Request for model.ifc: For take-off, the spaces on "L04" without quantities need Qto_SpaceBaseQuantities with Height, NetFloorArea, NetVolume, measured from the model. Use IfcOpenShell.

First a look at what the model holds.

```python
import ifcopenshell
import ifcopenshell.util.element
import ifcopenshell.util.unit

model = ifcopenshell.open("model.ifc")
print(model.schema)
for unit_type in ("LENGTHUNIT", "AREAUNIT", "VOLUMEUNIT"):
    print(unit_type, ifcopenshell.util.unit.calculate_unit_scale(model, unit_type))
storey = next(s for s in model.by_type("IfcBuildingStorey") if s.Name == "L04")
spaces = [e for e in ifcopenshell.util.element.get_decomposition(storey) if e.is_a("IfcSpace")]
for e in sorted(spaces, key=lambda e: e.id()):
    print(e.id(), e.is_a(), e.Name, list(ifcopenshell.util.element.get_psets(e, qtos_only=True)), sep=" | ")
```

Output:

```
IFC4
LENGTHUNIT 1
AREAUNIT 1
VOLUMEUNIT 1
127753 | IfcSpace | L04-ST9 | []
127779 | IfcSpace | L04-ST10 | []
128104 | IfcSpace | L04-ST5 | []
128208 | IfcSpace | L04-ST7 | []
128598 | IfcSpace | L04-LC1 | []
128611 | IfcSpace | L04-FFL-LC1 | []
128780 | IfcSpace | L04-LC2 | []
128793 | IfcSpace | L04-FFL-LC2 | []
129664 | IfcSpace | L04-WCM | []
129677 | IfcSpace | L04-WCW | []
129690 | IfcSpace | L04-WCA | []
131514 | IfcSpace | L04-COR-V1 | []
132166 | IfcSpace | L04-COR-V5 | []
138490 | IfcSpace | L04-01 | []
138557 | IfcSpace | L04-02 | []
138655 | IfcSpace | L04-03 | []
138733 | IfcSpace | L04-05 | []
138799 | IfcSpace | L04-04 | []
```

```python
import ifcopenshell
import ifcopenshell.api.pset
import ifcopenshell.geom
import ifcopenshell.util.element
import ifcopenshell.util.shape
import ifcopenshell.util.unit

model = ifcopenshell.open("model.ifc")
unit_scale = ifcopenshell.util.unit.calculate_unit_scale(model)
area_scale = ifcopenshell.util.unit.calculate_unit_scale(model, "AREAUNIT")
volume_scale = ifcopenshell.util.unit.calculate_unit_scale(model, "VOLUMEUNIT")
settings = ifcopenshell.geom.settings()

storey = next(s for s in model.by_type("IfcBuildingStorey") if s.Name == "L04")
spaces = [e for e in ifcopenshell.util.element.get_decomposition(storey) if e.is_a("IfcSpace")]

for e in sorted(spaces, key=lambda e: e.id()):
    if ifcopenshell.util.element.get_psets(e, qtos_only=True, should_inherit=False):
        continue
    # Geometry comes back in metres, in the element's own axes.
    shape = ifcopenshell.geom.create_shape(settings, e)
    values = {
        "Height": ifcopenshell.util.shape.get_z(shape.geometry) / unit_scale,
        "NetFloorArea": ifcopenshell.util.shape.get_footprint_area(shape.geometry) / area_scale,
        "NetVolume": ifcopenshell.util.shape.get_volume(shape.geometry) / volume_scale,
    }
    qto = ifcopenshell.api.pset.add_qto(model, product=e, name="Qto_SpaceBaseQuantities")
    ifcopenshell.api.pset.edit_qto(model, qto=qto, properties=values)
    print(e.id(), {k: round(v, 3) for k, v in values.items()})

model.write("model_v2.ifc")
```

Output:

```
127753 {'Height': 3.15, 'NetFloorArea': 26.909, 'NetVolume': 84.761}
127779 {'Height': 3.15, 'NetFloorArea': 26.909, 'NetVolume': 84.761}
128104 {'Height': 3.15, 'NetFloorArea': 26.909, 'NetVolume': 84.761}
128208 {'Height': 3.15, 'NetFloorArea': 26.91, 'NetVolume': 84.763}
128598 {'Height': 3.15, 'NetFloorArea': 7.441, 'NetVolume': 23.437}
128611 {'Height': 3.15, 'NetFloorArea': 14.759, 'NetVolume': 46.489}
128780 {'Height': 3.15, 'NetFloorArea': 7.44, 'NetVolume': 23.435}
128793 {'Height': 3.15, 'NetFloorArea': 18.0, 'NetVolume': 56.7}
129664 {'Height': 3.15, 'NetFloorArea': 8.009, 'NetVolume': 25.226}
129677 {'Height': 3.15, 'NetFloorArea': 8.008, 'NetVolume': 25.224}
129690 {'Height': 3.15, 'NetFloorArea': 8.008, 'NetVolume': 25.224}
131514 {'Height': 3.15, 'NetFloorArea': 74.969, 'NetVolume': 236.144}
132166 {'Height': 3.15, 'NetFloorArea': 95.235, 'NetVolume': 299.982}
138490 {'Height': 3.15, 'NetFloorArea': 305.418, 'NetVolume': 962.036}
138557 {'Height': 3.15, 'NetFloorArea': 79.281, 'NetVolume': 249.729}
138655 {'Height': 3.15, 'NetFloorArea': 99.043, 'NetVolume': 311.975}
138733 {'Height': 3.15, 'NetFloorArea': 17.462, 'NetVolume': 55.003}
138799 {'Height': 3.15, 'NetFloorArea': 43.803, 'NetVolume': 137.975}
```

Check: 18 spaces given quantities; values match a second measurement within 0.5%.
